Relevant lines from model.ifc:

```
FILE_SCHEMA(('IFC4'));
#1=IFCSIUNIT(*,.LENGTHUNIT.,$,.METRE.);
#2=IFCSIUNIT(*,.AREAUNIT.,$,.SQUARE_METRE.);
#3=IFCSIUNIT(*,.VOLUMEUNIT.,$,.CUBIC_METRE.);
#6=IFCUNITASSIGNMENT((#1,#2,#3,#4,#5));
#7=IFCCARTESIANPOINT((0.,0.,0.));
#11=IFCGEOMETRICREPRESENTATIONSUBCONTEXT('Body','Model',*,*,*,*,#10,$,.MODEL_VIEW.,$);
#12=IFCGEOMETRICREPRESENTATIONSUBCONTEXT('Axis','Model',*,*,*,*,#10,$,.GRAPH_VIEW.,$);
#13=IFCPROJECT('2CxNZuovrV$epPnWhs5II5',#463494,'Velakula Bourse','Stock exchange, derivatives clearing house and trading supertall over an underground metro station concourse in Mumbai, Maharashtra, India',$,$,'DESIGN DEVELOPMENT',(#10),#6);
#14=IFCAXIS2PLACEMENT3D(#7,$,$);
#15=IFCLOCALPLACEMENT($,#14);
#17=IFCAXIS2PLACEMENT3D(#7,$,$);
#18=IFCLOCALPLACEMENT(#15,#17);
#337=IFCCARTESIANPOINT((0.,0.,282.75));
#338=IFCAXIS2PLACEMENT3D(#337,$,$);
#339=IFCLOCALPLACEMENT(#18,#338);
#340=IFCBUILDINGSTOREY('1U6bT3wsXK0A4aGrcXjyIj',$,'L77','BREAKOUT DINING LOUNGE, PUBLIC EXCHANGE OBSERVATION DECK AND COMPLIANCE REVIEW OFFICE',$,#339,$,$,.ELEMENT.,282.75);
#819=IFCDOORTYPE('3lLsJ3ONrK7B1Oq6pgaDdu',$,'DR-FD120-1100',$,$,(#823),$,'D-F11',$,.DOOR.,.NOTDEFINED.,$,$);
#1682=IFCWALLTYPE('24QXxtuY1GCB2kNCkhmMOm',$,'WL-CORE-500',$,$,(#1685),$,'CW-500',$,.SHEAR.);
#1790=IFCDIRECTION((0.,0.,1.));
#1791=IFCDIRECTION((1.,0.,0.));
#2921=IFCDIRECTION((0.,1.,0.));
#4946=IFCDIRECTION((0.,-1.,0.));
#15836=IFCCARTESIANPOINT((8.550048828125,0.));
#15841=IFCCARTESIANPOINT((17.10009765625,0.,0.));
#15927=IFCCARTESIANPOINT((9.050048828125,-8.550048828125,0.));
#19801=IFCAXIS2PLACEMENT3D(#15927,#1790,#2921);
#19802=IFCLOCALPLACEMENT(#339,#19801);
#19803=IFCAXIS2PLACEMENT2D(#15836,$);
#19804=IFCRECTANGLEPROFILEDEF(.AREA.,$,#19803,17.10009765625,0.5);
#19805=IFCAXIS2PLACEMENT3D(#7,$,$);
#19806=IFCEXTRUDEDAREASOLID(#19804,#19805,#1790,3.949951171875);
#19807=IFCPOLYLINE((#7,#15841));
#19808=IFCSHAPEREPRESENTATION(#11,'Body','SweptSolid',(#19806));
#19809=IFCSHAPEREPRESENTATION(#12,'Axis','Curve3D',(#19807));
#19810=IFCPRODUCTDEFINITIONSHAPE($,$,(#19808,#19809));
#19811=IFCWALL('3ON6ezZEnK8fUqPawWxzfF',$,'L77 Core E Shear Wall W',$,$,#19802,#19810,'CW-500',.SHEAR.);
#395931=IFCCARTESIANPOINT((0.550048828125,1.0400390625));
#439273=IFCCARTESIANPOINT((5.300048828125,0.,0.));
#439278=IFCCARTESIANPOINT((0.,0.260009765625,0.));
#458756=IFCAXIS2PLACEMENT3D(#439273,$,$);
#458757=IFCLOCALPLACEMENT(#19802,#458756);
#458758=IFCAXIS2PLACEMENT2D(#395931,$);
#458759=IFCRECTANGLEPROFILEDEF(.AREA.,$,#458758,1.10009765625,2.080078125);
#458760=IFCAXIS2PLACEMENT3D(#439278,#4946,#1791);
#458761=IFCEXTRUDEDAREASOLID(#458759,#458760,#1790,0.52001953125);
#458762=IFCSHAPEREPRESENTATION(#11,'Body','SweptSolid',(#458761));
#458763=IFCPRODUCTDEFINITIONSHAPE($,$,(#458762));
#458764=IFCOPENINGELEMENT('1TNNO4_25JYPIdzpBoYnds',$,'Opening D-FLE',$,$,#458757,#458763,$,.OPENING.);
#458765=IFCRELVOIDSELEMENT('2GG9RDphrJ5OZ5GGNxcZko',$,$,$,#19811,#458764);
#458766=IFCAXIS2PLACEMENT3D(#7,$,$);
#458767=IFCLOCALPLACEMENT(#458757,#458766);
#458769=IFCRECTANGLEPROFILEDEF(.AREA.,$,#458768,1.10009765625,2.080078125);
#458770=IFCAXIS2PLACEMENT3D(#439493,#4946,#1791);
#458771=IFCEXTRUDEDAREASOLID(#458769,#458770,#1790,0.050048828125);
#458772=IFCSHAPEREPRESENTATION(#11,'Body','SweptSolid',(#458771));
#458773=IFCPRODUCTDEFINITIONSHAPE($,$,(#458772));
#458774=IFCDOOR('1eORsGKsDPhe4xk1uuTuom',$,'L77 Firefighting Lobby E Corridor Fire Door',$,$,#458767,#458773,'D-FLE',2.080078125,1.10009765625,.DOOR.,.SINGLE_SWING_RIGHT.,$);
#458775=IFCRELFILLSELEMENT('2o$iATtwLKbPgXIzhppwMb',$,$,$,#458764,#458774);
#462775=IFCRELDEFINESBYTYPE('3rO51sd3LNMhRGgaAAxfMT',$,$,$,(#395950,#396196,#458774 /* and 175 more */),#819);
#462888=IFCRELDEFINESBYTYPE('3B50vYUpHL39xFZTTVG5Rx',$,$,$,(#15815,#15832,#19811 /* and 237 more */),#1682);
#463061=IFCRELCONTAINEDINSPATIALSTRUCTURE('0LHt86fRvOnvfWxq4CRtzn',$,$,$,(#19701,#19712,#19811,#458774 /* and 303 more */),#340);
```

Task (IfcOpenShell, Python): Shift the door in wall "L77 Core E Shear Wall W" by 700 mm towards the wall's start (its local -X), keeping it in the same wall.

```python
import ifcopenshell
import ifcopenshell.api.geometry
import ifcopenshell.util.placement

model = ifcopenshell.open("model.ifc")

door = model.by_guid("1eORsGKsDPhe4xk1uuTuom")
opening = door.FillsVoids[0].RelatingOpeningElement
wall = opening.VoidsElements[0].RelatingBuildingElement

wall_matrix = ifcopenshell.util.placement.get_local_placement(wall.ObjectPlacement)
shift = wall_matrix[:3, 0] * -0.7
before = ifcopenshell.util.placement.get_local_placement(door.ObjectPlacement)[:3, 3].copy()

# The door is placed relative to its opening, so it follows when the opening moves.
matrix = ifcopenshell.util.placement.get_local_placement(opening.ObjectPlacement)
matrix[:3, 3] += shift
ifcopenshell.api.geometry.edit_object_placement(
    model, product=opening, matrix=matrix, is_si=False, should_transform_children=True
)

after = ifcopenshell.util.placement.get_local_placement(door.ObjectPlacement)[:3, 3]
print("door moved by", (after - before).round(3) + 0.0)

model.write("model_updated.ifc")
```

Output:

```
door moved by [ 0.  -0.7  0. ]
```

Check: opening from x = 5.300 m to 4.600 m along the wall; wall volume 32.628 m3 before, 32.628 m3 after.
